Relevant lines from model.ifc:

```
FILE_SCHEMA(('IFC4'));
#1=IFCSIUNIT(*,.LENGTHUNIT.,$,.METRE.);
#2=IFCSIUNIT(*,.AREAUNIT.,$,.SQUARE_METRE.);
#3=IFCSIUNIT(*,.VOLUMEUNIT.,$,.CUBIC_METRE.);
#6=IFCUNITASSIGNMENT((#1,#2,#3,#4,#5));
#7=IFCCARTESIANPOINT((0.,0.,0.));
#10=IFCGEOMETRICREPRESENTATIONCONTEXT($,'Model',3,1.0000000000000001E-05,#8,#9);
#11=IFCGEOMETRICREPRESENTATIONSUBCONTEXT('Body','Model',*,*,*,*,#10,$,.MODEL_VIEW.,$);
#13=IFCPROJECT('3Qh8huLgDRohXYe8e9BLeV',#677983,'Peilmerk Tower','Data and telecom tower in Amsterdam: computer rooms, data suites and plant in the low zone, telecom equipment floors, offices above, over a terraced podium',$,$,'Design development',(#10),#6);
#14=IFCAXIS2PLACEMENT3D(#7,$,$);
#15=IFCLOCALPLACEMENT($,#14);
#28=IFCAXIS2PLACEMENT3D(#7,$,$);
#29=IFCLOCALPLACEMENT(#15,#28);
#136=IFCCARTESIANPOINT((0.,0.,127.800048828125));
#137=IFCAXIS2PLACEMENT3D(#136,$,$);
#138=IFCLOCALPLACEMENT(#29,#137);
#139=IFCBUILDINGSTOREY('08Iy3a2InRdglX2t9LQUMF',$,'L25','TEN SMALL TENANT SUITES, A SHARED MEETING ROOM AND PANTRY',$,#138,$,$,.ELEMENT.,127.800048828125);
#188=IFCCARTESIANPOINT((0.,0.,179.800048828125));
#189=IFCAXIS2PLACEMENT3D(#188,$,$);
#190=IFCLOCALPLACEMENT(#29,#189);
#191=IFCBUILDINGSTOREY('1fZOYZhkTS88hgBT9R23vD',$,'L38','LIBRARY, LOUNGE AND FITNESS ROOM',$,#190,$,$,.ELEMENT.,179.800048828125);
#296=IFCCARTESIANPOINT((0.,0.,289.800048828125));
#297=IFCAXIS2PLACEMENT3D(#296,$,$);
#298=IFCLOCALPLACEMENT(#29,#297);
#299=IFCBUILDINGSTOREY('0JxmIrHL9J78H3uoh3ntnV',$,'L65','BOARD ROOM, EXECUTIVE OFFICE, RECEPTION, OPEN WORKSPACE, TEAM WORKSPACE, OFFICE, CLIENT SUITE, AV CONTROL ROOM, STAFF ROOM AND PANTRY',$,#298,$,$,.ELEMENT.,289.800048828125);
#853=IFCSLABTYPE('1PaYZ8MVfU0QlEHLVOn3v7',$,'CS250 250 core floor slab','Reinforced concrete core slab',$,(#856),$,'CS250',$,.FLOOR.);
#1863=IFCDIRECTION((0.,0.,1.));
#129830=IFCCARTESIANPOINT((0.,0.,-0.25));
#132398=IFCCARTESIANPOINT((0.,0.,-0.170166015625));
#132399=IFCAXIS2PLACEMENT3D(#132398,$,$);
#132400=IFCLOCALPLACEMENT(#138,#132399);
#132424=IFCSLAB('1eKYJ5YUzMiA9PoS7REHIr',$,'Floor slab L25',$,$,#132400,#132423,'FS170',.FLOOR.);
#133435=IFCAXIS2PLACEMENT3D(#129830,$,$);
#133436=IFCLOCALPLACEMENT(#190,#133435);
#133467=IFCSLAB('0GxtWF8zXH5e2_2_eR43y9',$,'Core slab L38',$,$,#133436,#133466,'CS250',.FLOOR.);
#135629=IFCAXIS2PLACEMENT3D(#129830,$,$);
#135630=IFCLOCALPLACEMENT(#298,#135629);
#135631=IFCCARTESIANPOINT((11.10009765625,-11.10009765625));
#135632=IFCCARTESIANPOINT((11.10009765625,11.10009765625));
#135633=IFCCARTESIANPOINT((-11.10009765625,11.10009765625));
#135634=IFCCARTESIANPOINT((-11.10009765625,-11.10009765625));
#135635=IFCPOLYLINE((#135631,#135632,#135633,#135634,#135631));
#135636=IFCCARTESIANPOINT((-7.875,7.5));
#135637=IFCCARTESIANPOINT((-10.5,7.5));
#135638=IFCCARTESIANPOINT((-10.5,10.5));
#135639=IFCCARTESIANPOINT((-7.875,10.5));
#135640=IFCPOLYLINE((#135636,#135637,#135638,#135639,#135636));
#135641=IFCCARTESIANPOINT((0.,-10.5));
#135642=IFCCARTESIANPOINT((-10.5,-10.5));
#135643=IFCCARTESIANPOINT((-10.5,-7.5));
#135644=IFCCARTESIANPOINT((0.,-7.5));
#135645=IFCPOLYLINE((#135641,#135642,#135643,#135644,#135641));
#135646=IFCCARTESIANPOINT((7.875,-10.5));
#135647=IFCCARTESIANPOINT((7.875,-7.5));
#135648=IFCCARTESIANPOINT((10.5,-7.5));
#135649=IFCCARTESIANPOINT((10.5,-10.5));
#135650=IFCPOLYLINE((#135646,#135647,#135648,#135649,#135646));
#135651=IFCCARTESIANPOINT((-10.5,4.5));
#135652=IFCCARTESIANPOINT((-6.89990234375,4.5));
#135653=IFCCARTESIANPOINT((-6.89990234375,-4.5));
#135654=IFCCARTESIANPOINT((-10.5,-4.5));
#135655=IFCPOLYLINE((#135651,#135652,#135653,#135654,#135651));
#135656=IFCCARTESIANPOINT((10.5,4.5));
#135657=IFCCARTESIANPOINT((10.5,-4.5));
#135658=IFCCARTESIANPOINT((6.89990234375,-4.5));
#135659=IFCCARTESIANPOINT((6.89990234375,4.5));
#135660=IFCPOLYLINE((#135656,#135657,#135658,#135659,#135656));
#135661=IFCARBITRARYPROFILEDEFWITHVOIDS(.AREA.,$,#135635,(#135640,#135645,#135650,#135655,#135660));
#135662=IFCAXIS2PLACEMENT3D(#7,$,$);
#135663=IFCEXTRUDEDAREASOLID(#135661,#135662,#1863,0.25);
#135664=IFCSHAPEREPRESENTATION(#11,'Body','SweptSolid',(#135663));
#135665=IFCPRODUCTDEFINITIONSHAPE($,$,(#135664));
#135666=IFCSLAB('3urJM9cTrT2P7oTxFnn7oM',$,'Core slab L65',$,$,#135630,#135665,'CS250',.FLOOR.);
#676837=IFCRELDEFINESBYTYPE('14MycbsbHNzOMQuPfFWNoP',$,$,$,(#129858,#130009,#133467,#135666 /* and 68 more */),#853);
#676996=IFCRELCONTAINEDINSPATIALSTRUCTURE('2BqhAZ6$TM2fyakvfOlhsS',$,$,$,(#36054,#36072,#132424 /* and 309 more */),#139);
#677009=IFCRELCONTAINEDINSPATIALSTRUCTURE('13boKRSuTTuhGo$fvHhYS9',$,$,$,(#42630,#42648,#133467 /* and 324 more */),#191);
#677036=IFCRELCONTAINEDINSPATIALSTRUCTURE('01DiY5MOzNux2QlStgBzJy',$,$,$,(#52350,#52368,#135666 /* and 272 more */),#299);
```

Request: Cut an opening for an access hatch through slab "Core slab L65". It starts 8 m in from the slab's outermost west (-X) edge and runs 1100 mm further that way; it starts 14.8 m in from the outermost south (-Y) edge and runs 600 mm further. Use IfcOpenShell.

```python
import numpy as np
import ifcopenshell
import ifcopenshell.api.feature
import ifcopenshell.api.geometry
import ifcopenshell.api.root
import ifcopenshell.geom
import ifcopenshell.util.placement
import ifcopenshell.util.representation
import ifcopenshell.util.shape
import ifcopenshell.util.unit

model = ifcopenshell.open("model.ifc")
unit_scale = ifcopenshell.util.unit.calculate_unit_scale(model)
settings = ifcopenshell.geom.settings()


def volume(element):
    """Net volume in cubic metres, openings subtracted."""
    shape = ifcopenshell.geom.create_shape(settings, element)
    return ifcopenshell.util.shape.get_volume(shape.geometry)


slab = model.by_guid("3urJM9cTrT2P7oTxFnn7oM")
before = volume(slab)

# Extent in the slab's own axes, in metres. The edges named are its -X and -Y sides.
slab_shape = ifcopenshell.geom.create_shape(settings, slab)
vertices = ifcopenshell.util.shape.get_vertices(slab_shape.geometry)
x_min, y_min, bottom = vertices.min(axis=0)
top = vertices[:, 2].max()

opening = ifcopenshell.api.root.create_entity(model, ifc_class="IfcOpeningElement", name="Access hatch opening", predefined_type="OPENING")
context = ifcopenshell.util.representation.get_context(model, "Model", "Body", "MODEL_VIEW")
width, depth = 1.1, 0.6
outline = [(0.0, 0.0), (width, 0.0), (width, depth), (0.0, depth), (0.0, 0.0)]
# Overshoot both faces by 50 mm so the cut is clean.
shape = ifcopenshell.api.geometry.add_slab_representation(
    model, context=context, depth=top - bottom + 0.1, polyline=outline
)
ifcopenshell.api.geometry.assign_representation(model, product=opening, representation=shape)

matrix = ifcopenshell.util.placement.get_local_placement(slab.ObjectPlacement)
matrix[:, 3] = matrix @ np.append(np.array([x_min + 8, y_min + 14.8, bottom - 0.05]) / unit_scale, 1.0)
ifcopenshell.api.geometry.edit_object_placement(model, product=opening, matrix=matrix, is_si=False)
ifcopenshell.api.feature.add_feature(model, feature=opening, element=slab)

after = volume(slab)

print(f"slab volume {before:.3f} -> {after:.3f} m3")

model.write("model_updated.ifc")
```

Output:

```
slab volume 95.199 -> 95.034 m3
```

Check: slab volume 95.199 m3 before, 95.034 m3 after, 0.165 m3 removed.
